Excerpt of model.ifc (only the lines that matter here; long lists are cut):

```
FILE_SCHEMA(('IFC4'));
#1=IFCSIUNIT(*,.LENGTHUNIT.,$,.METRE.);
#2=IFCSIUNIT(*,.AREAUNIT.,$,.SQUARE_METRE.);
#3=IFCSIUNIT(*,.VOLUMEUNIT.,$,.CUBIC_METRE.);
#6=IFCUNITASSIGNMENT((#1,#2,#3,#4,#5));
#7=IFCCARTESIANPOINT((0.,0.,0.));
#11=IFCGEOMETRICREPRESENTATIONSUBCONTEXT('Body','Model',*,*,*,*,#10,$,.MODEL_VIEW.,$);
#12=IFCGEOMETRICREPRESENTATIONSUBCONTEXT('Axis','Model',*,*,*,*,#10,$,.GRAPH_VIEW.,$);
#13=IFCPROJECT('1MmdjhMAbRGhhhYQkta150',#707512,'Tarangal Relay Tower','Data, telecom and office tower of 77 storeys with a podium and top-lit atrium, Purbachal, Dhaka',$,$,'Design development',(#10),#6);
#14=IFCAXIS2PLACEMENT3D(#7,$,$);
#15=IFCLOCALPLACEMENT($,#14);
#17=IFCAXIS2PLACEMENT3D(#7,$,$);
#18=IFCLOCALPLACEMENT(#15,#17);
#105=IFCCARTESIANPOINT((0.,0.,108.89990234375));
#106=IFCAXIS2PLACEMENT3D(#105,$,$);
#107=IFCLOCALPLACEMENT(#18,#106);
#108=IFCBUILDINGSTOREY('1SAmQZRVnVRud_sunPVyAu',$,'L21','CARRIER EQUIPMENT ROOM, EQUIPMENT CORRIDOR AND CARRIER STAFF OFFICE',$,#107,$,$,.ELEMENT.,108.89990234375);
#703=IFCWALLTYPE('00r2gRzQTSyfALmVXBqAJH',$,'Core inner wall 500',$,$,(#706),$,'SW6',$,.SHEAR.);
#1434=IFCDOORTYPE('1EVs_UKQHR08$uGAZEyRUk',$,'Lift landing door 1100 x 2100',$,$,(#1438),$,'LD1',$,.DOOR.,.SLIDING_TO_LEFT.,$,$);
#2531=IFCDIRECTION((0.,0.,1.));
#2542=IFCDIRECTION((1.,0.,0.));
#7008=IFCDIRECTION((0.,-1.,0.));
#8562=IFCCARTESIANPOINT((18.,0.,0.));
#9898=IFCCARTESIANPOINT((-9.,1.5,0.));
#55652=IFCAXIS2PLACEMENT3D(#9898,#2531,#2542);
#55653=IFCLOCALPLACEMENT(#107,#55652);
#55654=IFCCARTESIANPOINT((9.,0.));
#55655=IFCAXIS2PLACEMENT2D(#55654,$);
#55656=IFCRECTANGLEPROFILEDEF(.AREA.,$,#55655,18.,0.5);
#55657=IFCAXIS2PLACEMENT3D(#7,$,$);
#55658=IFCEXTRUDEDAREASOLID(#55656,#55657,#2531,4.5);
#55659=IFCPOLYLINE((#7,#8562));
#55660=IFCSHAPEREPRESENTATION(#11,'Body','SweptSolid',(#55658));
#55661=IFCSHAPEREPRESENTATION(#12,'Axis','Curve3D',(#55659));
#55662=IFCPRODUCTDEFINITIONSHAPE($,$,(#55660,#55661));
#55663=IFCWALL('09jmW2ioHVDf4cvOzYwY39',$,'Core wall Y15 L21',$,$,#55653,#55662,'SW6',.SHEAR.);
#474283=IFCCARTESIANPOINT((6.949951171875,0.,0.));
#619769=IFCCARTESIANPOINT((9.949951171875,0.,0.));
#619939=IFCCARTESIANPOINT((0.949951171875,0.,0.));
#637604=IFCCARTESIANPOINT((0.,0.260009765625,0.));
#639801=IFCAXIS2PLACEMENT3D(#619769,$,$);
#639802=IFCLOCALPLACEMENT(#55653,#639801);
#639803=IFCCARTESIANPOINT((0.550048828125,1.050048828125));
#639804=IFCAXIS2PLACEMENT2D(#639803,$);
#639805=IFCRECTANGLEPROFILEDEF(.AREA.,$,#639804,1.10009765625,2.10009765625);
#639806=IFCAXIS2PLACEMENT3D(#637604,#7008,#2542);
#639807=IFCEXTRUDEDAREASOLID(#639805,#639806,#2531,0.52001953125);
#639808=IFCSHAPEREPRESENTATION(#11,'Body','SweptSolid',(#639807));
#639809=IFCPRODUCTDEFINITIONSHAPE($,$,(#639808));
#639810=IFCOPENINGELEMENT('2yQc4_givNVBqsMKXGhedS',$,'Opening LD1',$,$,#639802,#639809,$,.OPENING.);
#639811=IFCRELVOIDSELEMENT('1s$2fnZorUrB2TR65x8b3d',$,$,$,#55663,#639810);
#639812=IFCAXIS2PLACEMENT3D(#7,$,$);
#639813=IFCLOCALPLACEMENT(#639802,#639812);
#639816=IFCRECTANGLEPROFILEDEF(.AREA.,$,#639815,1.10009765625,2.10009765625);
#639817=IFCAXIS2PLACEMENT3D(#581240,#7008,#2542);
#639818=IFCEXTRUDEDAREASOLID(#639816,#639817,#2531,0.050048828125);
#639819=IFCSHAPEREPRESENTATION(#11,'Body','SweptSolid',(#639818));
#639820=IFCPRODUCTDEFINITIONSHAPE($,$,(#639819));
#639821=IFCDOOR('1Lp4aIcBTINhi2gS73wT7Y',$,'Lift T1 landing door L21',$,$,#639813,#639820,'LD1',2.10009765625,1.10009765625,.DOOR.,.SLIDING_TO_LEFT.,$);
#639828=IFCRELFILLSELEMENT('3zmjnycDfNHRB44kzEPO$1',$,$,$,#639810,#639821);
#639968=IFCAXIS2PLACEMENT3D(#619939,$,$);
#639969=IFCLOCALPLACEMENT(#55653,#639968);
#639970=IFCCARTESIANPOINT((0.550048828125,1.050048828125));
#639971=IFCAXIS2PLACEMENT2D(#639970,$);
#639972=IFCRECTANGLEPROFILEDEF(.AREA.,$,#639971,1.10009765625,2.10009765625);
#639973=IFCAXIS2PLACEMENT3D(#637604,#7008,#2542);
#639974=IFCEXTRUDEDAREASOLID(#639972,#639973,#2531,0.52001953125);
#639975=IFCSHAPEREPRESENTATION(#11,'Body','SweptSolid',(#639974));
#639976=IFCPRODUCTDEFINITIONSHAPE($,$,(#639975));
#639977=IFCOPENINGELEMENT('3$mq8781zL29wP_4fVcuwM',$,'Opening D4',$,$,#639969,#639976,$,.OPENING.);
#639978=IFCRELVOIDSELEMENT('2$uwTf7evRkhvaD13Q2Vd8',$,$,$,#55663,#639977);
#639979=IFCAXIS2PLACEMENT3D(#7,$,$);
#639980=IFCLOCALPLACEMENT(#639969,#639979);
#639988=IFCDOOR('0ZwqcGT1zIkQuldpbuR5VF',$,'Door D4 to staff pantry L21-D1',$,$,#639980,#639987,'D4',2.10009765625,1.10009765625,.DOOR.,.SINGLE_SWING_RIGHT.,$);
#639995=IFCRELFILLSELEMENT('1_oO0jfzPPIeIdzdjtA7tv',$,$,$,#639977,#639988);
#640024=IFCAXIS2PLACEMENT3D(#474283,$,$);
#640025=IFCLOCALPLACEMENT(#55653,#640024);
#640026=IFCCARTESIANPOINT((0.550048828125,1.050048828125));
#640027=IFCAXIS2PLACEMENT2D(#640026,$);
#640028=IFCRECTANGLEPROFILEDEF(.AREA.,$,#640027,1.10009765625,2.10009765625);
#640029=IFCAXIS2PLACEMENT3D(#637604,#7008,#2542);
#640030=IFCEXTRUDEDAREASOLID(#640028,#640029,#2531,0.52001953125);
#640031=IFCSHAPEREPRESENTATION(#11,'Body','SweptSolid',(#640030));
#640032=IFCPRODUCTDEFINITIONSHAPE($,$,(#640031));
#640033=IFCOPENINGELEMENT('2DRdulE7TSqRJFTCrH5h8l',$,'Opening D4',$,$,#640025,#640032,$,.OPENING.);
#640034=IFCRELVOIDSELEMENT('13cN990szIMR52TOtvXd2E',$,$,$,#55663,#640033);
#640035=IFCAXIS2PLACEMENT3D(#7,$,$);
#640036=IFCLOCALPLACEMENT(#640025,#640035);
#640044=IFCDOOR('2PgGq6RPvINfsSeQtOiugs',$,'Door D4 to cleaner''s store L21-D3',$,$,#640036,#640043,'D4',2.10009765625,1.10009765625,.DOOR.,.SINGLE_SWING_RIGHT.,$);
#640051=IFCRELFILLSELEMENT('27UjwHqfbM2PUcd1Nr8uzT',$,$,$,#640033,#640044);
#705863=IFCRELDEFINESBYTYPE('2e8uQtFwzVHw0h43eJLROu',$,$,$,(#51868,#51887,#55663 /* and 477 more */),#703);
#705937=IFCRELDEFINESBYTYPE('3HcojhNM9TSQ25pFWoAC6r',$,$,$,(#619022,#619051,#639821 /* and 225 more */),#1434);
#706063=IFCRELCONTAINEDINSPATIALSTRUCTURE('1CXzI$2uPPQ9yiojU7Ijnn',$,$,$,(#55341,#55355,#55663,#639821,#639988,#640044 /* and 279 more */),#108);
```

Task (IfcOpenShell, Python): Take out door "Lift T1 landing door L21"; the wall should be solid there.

```python
import ifcopenshell
import ifcopenshell.api.feature
import ifcopenshell.api.root
import ifcopenshell.geom
import ifcopenshell.util.shape

model = ifcopenshell.open("model.ifc")
settings = ifcopenshell.geom.settings()


def volume(element):
    """Net volume in cubic metres, openings subtracted."""
    shape = ifcopenshell.geom.create_shape(settings, element)
    return ifcopenshell.util.shape.get_volume(shape.geometry)


door = model.by_guid("1Lp4aIcBTINhi2gS73wT7Y")
opening = door.FillsVoids[0].RelatingOpeningElement
wall = opening.VoidsElements[0].RelatingBuildingElement
before = volume(wall)

ifcopenshell.api.root.remove_product(model, product=door)
ifcopenshell.api.feature.remove_feature(model, feature=opening)

after = volume(wall)

print(f"wall volume {before:.3f} -> {after:.3f} m3")

model.write("model_edited.ifc")
```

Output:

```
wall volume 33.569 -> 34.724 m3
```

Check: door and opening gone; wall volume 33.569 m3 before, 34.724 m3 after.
